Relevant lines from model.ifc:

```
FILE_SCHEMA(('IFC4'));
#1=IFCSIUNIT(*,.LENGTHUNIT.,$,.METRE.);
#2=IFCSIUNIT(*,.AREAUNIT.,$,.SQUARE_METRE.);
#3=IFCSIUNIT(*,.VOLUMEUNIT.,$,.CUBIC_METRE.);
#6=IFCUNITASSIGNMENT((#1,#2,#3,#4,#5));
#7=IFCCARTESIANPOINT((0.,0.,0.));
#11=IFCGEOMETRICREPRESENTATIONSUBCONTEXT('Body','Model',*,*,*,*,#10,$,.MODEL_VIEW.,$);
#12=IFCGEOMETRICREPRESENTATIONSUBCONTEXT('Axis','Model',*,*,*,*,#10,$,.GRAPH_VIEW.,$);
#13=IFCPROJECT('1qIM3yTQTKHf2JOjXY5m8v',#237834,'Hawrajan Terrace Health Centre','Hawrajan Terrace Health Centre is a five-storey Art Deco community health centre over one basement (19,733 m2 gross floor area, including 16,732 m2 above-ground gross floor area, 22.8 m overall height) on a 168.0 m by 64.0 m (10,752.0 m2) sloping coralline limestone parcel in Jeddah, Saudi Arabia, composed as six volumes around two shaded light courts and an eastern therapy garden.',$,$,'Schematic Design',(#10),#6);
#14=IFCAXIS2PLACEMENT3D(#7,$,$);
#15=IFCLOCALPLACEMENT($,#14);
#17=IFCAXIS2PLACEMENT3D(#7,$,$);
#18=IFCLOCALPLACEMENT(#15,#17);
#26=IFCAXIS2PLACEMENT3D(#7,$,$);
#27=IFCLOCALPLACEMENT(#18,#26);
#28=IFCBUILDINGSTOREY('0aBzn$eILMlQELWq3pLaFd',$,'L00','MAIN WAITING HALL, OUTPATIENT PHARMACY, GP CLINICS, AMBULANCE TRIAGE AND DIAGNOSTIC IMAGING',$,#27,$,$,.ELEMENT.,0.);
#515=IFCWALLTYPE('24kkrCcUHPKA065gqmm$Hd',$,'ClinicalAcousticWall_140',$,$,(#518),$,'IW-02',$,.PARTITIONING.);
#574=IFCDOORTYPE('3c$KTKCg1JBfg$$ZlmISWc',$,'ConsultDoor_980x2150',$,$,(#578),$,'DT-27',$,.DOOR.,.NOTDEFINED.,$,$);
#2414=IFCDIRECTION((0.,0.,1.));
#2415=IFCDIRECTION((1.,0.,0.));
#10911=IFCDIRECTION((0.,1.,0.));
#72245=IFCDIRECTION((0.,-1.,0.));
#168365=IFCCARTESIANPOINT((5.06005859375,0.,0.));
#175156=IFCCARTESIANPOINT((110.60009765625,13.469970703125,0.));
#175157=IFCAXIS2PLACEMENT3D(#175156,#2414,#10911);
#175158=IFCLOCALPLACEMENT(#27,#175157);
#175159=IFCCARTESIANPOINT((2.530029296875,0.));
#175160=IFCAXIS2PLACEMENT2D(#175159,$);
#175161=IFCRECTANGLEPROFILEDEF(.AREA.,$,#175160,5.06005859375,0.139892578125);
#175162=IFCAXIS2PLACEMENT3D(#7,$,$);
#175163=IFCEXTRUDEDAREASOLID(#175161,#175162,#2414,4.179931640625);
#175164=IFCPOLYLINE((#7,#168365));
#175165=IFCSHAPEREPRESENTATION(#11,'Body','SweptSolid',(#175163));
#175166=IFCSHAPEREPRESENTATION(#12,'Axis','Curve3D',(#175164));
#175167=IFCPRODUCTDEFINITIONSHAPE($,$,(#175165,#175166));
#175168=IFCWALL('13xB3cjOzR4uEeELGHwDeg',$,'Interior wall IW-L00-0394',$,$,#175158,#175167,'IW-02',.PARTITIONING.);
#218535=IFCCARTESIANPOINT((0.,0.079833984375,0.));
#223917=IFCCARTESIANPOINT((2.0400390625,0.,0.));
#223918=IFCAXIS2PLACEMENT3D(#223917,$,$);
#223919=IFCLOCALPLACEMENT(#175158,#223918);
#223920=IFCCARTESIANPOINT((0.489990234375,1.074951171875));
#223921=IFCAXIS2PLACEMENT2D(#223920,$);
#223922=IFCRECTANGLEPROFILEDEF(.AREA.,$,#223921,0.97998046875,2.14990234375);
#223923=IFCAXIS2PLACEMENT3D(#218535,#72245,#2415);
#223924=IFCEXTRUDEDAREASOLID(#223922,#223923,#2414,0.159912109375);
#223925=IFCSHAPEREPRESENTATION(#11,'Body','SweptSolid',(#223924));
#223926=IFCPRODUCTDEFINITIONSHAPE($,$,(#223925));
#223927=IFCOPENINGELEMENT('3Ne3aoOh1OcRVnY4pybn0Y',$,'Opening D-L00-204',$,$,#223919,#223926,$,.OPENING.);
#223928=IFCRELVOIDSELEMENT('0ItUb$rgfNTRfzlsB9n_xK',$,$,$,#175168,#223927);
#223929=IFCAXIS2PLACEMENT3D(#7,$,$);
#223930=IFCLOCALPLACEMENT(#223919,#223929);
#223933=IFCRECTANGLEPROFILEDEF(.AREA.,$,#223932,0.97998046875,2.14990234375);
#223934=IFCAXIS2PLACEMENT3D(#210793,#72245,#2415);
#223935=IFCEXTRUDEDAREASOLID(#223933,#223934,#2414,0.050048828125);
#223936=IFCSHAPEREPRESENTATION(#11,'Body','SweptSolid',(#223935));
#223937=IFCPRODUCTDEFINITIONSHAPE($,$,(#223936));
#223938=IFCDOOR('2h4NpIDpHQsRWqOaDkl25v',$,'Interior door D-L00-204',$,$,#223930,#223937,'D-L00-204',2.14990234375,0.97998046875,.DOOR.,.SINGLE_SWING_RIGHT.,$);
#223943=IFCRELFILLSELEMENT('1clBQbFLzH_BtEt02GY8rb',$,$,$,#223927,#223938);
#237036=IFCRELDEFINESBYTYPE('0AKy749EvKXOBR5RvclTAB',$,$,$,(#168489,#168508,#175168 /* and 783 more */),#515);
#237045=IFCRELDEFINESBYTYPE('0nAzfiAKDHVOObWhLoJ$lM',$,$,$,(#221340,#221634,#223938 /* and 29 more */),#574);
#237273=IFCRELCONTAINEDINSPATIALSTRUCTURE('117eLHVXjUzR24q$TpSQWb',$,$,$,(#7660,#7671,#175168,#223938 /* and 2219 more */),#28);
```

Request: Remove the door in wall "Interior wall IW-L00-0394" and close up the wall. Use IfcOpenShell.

```python
import ifcopenshell
import ifcopenshell.api.feature
import ifcopenshell.api.root
import ifcopenshell.geom
import ifcopenshell.util.shape

model = ifcopenshell.open("model.ifc")
settings = ifcopenshell.geom.settings()


def volume(element):
    """Net volume in cubic metres, openings subtracted."""
    shape = ifcopenshell.geom.create_shape(settings, element)
    return ifcopenshell.util.shape.get_volume(shape.geometry)


door = model.by_id(223938)
opening = door.FillsVoids[0].RelatingOpeningElement
wall = opening.VoidsElements[0].RelatingBuildingElement
before = volume(wall)

ifcopenshell.api.root.remove_product(model, product=door)
ifcopenshell.api.feature.remove_feature(model, feature=opening)

after = volume(wall)

print(f"wall volume {before:.3f} -> {after:.3f} m3")

model.write("model_edited.ifc")
```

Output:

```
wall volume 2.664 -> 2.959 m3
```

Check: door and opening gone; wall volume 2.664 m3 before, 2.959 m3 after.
